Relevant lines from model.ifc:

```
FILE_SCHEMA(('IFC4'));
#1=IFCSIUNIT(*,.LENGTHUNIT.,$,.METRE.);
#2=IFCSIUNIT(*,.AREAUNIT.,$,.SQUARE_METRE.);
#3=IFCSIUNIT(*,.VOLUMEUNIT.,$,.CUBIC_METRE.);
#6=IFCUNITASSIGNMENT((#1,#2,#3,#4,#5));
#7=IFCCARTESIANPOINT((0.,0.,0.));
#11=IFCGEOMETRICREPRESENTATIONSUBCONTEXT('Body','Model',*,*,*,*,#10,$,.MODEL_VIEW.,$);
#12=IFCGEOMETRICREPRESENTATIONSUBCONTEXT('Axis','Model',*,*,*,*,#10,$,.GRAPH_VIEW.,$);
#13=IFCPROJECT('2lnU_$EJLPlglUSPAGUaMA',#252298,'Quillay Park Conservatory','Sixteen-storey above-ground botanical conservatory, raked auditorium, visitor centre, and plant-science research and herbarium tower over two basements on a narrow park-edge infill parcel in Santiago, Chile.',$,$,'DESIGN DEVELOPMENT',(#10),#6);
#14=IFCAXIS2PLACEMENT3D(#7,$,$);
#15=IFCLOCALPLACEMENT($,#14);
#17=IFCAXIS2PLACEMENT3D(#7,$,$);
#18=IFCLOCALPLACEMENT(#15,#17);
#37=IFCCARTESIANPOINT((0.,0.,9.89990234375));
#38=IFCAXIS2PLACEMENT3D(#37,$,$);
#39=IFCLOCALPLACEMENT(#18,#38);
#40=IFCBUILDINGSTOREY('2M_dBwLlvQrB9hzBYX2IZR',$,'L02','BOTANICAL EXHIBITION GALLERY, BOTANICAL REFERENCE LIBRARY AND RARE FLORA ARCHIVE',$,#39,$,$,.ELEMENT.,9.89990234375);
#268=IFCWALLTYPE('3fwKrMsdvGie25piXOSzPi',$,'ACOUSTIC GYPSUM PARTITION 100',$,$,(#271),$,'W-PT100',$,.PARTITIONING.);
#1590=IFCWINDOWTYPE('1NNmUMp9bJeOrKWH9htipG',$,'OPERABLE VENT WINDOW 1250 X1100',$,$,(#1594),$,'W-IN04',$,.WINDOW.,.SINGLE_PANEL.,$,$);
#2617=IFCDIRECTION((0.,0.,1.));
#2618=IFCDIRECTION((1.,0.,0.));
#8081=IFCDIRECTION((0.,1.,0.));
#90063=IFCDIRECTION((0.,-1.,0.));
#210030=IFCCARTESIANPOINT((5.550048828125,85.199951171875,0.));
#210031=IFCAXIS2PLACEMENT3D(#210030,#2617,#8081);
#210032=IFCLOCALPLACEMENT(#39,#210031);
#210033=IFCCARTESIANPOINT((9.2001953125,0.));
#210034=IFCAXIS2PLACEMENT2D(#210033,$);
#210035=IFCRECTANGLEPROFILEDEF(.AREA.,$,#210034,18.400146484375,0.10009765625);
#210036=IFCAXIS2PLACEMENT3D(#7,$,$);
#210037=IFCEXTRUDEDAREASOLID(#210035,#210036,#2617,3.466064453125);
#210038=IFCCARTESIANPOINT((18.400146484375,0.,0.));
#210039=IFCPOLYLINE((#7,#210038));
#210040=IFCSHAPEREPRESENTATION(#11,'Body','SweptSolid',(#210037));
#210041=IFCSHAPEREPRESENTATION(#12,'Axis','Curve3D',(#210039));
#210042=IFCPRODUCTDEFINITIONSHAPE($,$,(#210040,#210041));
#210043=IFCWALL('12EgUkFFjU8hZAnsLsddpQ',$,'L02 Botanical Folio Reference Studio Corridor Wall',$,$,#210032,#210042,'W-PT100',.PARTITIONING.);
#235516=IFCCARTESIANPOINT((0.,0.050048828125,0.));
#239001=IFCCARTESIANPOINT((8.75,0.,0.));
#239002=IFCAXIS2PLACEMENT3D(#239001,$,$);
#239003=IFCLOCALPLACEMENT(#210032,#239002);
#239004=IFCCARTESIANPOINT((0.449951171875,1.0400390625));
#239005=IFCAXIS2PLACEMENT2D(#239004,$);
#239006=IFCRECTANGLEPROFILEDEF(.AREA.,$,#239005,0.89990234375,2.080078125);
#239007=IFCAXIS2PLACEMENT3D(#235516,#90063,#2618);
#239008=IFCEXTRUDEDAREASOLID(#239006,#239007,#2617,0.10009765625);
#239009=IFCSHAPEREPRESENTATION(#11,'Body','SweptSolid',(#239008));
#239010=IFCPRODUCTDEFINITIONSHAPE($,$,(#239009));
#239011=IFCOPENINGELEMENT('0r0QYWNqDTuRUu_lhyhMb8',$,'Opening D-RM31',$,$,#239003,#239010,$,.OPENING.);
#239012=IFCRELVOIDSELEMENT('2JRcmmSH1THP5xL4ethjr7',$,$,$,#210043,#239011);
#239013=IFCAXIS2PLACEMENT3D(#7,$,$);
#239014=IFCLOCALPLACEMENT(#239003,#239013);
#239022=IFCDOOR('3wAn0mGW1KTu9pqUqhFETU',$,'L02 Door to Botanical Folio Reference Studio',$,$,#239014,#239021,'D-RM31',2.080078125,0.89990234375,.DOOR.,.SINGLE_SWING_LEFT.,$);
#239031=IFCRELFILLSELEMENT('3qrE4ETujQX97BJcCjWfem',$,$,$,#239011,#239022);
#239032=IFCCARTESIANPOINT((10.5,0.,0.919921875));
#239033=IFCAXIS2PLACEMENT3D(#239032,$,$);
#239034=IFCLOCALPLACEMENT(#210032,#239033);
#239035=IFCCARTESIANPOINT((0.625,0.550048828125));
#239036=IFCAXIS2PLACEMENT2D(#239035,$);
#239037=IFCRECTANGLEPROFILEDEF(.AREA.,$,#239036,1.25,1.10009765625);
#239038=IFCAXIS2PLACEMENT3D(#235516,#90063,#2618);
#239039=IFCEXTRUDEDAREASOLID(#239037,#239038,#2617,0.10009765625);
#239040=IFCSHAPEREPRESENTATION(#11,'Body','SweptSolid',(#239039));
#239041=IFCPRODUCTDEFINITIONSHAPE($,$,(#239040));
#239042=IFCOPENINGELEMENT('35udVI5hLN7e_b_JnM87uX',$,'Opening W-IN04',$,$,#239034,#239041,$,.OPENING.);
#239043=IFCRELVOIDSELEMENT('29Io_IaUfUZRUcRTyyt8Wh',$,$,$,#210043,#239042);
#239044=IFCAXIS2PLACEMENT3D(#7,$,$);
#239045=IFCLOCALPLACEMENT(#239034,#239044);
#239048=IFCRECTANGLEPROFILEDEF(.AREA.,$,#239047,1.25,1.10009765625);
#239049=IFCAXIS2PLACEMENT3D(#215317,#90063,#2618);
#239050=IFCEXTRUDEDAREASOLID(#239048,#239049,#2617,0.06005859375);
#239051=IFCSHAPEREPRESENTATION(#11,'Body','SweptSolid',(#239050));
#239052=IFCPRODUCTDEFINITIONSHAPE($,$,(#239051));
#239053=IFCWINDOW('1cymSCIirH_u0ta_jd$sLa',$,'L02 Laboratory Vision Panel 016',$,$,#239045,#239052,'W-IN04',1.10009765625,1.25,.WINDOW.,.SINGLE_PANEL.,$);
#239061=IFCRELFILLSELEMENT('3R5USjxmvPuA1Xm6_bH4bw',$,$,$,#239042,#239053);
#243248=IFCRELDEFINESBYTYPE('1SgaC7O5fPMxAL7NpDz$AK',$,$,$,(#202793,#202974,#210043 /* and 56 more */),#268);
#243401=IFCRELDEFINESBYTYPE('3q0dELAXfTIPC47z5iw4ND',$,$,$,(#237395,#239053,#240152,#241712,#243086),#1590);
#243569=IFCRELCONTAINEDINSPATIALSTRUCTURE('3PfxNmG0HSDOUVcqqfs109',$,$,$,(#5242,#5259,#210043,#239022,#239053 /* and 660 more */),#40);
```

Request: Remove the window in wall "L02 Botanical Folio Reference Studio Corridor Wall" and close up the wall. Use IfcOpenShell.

```python
import ifcopenshell
import ifcopenshell.api.feature
import ifcopenshell.api.root
import ifcopenshell.geom
import ifcopenshell.util.shape

model = ifcopenshell.open("model.ifc")
settings = ifcopenshell.geom.settings()


def volume(element):
    """Net volume in cubic metres, openings subtracted."""
    shape = ifcopenshell.geom.create_shape(settings, element)
    return ifcopenshell.util.shape.get_volume(shape.geometry)


window = model.by_guid("1cymSCIirH_u0ta_jd$sLa")
opening = window.FillsVoids[0].RelatingOpeningElement
wall = opening.VoidsElements[0].RelatingBuildingElement
before = volume(wall)

ifcopenshell.api.root.remove_product(model, product=window)
ifcopenshell.api.feature.remove_feature(model, feature=opening)

after = volume(wall)

print(f"wall volume {before:.3f} -> {after:.3f} m3")

model.write("model-out.ifc")
```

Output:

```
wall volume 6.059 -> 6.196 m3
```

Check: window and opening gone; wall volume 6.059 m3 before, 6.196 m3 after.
